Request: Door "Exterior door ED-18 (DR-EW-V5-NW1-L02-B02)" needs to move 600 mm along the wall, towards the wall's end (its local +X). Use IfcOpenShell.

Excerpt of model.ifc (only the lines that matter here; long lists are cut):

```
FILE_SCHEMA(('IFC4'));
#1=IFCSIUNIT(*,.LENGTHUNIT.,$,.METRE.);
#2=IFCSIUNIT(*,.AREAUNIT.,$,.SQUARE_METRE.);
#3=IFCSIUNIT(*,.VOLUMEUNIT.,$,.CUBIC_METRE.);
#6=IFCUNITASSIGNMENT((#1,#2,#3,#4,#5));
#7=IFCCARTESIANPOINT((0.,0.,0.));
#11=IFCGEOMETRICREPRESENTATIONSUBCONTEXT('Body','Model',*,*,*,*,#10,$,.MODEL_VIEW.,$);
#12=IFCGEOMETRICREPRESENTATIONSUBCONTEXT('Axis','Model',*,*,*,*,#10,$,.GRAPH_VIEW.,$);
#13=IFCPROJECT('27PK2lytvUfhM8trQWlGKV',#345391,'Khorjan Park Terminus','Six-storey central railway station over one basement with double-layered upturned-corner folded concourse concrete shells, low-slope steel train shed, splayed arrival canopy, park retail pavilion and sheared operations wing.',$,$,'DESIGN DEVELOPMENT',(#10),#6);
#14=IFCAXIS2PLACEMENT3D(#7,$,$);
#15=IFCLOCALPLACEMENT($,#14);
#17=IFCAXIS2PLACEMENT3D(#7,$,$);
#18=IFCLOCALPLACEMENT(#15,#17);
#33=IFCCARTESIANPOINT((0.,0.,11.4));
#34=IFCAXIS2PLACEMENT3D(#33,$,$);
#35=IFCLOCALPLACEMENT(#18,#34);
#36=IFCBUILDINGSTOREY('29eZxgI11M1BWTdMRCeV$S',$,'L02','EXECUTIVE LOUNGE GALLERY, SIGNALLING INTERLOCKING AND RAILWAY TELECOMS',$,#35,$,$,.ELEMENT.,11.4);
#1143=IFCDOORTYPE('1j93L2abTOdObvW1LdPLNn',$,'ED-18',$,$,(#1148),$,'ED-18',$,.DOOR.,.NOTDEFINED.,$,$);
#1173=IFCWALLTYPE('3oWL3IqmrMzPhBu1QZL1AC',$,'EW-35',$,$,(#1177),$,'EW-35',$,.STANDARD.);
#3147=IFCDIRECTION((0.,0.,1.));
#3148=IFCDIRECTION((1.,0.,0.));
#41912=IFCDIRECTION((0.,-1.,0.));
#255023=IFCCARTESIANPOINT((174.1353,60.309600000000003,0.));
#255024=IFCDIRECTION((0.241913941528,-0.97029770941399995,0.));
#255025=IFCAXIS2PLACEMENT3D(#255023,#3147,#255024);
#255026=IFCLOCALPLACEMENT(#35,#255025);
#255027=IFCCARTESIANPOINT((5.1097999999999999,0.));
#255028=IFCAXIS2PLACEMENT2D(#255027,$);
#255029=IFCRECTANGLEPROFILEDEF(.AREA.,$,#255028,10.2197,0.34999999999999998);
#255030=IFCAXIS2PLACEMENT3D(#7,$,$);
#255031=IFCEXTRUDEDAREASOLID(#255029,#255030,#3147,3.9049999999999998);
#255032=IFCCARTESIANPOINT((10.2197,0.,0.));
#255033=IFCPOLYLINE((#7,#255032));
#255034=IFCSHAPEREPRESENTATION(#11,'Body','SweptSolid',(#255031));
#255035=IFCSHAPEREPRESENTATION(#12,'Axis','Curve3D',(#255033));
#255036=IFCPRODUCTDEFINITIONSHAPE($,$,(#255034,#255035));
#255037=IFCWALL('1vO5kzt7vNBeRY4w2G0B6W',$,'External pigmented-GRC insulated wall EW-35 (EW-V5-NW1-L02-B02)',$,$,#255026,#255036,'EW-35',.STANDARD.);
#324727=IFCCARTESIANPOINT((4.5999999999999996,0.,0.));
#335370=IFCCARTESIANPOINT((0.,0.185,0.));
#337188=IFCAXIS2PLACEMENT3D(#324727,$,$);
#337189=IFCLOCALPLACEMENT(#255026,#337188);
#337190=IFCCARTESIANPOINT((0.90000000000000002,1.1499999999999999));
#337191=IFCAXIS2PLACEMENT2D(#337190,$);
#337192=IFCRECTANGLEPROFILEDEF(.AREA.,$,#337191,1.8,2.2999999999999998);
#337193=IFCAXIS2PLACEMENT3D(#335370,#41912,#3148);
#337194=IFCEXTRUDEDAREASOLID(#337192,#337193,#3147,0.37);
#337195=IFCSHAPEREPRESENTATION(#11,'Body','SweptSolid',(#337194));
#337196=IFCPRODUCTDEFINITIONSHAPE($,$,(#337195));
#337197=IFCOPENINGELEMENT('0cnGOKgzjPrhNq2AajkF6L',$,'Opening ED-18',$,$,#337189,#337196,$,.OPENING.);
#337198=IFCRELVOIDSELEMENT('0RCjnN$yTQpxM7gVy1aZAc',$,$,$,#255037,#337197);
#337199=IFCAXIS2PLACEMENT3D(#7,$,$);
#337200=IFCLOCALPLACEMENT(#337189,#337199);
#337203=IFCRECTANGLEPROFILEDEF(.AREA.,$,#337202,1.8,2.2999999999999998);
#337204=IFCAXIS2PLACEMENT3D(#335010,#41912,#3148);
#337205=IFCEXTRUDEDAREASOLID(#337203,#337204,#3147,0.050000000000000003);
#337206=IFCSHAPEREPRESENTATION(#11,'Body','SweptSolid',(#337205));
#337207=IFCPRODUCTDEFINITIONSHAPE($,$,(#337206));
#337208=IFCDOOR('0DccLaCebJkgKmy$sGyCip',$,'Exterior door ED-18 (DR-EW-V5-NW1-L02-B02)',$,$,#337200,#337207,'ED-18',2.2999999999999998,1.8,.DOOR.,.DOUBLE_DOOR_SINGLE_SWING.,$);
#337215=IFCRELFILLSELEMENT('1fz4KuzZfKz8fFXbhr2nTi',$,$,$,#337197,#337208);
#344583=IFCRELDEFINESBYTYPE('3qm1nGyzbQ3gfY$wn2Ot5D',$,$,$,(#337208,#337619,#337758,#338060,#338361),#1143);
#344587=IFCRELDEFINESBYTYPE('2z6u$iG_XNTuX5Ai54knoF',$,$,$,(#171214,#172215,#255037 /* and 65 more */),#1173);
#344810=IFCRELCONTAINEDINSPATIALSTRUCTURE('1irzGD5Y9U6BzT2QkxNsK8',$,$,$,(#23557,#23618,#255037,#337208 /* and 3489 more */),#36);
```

```python
import ifcopenshell
import ifcopenshell.api.geometry
import ifcopenshell.util.placement

model = ifcopenshell.open("model.ifc")

door = model.by_guid("0DccLaCebJkgKmy$sGyCip")
opening = door.FillsVoids[0].RelatingOpeningElement
wall = opening.VoidsElements[0].RelatingBuildingElement

wall_matrix = ifcopenshell.util.placement.get_local_placement(wall.ObjectPlacement)
shift = wall_matrix[:3, 0] * 0.6
before = ifcopenshell.util.placement.get_local_placement(door.ObjectPlacement)[:3, 3].copy()

# The door is placed relative to its opening, so it follows when the opening moves.
matrix = ifcopenshell.util.placement.get_local_placement(opening.ObjectPlacement)
matrix[:3, 3] += shift
ifcopenshell.api.geometry.edit_object_placement(
    model, product=opening, matrix=matrix, is_si=False, should_transform_children=True
)

after = ifcopenshell.util.placement.get_local_placement(door.ObjectPlacement)[:3, 3]
print("door moved by", (after - before).round(3) + 0.0)

model.write("model_updated.ifc")
```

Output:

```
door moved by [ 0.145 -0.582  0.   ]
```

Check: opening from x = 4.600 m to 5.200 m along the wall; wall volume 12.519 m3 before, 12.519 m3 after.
